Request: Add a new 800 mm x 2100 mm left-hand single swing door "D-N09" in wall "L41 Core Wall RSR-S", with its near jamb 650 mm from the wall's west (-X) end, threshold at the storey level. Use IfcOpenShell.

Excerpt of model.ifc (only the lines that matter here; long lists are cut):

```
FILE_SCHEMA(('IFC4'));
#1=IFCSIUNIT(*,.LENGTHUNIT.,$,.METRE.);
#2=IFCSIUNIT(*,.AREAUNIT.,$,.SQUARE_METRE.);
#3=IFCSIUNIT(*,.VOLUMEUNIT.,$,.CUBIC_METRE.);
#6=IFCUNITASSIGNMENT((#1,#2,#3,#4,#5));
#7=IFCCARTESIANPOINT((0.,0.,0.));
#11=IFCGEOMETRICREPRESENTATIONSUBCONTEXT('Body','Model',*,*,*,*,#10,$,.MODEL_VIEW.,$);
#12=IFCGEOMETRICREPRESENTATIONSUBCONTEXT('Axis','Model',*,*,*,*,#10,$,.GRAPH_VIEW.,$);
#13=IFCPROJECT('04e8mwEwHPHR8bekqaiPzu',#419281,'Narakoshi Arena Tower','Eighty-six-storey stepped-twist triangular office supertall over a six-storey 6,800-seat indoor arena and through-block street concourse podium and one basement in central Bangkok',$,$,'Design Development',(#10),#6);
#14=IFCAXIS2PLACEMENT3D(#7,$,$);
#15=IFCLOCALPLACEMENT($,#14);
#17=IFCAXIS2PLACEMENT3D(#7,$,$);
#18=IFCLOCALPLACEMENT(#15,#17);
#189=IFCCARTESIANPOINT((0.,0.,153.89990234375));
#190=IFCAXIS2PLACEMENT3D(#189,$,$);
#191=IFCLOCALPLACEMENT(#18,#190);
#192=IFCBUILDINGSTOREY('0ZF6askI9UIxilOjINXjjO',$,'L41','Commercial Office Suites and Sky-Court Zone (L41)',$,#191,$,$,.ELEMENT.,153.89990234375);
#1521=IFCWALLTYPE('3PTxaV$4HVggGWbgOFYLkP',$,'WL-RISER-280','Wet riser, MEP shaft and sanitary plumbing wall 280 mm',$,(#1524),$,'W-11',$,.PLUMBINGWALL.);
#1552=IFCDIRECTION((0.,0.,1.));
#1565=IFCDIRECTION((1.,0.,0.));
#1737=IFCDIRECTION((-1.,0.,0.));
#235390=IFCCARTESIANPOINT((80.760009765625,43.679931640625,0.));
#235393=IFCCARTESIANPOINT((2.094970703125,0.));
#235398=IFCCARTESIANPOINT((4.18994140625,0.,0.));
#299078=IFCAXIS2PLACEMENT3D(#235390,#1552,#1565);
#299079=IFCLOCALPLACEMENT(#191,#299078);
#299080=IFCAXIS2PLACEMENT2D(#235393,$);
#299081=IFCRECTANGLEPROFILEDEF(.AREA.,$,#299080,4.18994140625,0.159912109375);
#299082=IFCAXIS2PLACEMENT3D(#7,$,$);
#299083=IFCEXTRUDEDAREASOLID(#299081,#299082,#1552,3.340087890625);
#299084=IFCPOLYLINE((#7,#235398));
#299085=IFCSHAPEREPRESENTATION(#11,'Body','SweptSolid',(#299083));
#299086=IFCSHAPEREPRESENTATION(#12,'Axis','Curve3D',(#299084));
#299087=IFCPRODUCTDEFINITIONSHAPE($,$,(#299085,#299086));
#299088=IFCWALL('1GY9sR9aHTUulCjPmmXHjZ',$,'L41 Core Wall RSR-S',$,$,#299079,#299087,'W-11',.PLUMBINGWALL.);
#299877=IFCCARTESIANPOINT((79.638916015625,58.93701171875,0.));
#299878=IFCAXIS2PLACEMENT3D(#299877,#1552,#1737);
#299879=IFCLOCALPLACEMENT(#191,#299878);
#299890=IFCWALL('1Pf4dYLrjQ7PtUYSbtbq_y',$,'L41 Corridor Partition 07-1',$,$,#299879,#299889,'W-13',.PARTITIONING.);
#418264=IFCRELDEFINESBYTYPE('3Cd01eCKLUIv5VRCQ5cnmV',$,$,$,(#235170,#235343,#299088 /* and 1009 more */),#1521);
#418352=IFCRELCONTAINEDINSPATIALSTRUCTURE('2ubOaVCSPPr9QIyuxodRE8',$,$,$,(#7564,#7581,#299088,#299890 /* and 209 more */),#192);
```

```python
import numpy as np
import ifcopenshell
import ifcopenshell.api.feature
import ifcopenshell.api.geometry
import ifcopenshell.api.root
import ifcopenshell.api.spatial
import ifcopenshell.geom
import ifcopenshell.util.element
import ifcopenshell.util.placement
import ifcopenshell.util.representation
import ifcopenshell.util.shape
import ifcopenshell.util.unit

model = ifcopenshell.open("model.ifc")
unit_scale = ifcopenshell.util.unit.calculate_unit_scale(model)
settings = ifcopenshell.geom.settings()


def volume(element):
    """Net volume in cubic metres, openings subtracted."""
    shape = ifcopenshell.geom.create_shape(settings, element)
    return ifcopenshell.util.shape.get_volume(shape.geometry)


wall = model.by_guid("1GY9sR9aHTUulCjPmmXHjZ")
storey = ifcopenshell.util.element.get_container(wall, ifc_class="IfcBuildingStorey")
context = ifcopenshell.util.representation.get_context(model, "Model", "Body", "MODEL_VIEW")
before = volume(wall)

width, height, from_end, sill = 0.8, 2.1, 0.65, 0.0  # metres

# The wall runs along its own X axis, and the end named is its -X end.
wall_shape = ifcopenshell.geom.create_shape(settings, wall)
x, y, z = ifcopenshell.util.shape.get_vertices(wall_shape.geometry).T
start = x.min() + from_end
face, thickness = float(y.min()), float(y.max() - y.min())
wall_matrix = ifcopenshell.util.placement.get_local_placement(wall.ObjectPlacement)
level = ifcopenshell.util.placement.get_local_placement(storey.ObjectPlacement)[2, 3]


def in_wall(x, y):
    """Placement at x, y metres in the wall's axes, at sill height."""
    matrix = wall_matrix.copy()
    matrix[:, 3] = wall_matrix @ np.array([x / unit_scale, y / unit_scale, 0.0, 1.0])
    matrix[2, 3] = level + sill / unit_scale
    return matrix


# Opening: a box that overshoots both wall faces by 50 mm.
opening = ifcopenshell.api.root.create_entity(model, ifc_class="IfcOpeningElement", predefined_type="OPENING")
box = ifcopenshell.api.geometry.add_wall_representation(
    model, context=context, length=width, height=height, thickness=thickness + 0.1
)
ifcopenshell.api.geometry.assign_representation(model, product=opening, representation=box)
ifcopenshell.api.geometry.edit_object_placement(model, product=opening, matrix=in_wall(start, face - 0.05), is_si=False)
ifcopenshell.api.feature.add_feature(model, feature=opening, element=wall)

door = ifcopenshell.api.root.create_entity(model, ifc_class="IfcDoor", name="D-N09", predefined_type="DOOR")
door.OverallWidth, door.OverallHeight = width / unit_scale, height / unit_scale
door.OperationType = "SINGLE_SWING_LEFT"
body = ifcopenshell.api.geometry.add_door_representation(
    model,
    context=context,
    overall_width=door.OverallWidth,
    overall_height=door.OverallHeight,
    operation_type="SINGLE_SWING_LEFT",
    lining_properties={"LiningDepth": thickness / unit_scale, "ThresholdDepth": thickness / unit_scale},
)
ifcopenshell.api.geometry.assign_representation(model, product=door, representation=body)
ifcopenshell.api.spatial.assign_container(model, products=[door], relating_structure=storey)
ifcopenshell.api.feature.add_filling(model, opening=opening, element=door)

# The lining spans the wall, so the door starts at the wall face.
ifcopenshell.api.geometry.edit_object_placement(model, product=door, matrix=in_wall(start, face), is_si=False)

after = volume(wall)

print(f"wall volume {before:.3f} -> {after:.3f} m3")

model.write("model_v2.ifc")
```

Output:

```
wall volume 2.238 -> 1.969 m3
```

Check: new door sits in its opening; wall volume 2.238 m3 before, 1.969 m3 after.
